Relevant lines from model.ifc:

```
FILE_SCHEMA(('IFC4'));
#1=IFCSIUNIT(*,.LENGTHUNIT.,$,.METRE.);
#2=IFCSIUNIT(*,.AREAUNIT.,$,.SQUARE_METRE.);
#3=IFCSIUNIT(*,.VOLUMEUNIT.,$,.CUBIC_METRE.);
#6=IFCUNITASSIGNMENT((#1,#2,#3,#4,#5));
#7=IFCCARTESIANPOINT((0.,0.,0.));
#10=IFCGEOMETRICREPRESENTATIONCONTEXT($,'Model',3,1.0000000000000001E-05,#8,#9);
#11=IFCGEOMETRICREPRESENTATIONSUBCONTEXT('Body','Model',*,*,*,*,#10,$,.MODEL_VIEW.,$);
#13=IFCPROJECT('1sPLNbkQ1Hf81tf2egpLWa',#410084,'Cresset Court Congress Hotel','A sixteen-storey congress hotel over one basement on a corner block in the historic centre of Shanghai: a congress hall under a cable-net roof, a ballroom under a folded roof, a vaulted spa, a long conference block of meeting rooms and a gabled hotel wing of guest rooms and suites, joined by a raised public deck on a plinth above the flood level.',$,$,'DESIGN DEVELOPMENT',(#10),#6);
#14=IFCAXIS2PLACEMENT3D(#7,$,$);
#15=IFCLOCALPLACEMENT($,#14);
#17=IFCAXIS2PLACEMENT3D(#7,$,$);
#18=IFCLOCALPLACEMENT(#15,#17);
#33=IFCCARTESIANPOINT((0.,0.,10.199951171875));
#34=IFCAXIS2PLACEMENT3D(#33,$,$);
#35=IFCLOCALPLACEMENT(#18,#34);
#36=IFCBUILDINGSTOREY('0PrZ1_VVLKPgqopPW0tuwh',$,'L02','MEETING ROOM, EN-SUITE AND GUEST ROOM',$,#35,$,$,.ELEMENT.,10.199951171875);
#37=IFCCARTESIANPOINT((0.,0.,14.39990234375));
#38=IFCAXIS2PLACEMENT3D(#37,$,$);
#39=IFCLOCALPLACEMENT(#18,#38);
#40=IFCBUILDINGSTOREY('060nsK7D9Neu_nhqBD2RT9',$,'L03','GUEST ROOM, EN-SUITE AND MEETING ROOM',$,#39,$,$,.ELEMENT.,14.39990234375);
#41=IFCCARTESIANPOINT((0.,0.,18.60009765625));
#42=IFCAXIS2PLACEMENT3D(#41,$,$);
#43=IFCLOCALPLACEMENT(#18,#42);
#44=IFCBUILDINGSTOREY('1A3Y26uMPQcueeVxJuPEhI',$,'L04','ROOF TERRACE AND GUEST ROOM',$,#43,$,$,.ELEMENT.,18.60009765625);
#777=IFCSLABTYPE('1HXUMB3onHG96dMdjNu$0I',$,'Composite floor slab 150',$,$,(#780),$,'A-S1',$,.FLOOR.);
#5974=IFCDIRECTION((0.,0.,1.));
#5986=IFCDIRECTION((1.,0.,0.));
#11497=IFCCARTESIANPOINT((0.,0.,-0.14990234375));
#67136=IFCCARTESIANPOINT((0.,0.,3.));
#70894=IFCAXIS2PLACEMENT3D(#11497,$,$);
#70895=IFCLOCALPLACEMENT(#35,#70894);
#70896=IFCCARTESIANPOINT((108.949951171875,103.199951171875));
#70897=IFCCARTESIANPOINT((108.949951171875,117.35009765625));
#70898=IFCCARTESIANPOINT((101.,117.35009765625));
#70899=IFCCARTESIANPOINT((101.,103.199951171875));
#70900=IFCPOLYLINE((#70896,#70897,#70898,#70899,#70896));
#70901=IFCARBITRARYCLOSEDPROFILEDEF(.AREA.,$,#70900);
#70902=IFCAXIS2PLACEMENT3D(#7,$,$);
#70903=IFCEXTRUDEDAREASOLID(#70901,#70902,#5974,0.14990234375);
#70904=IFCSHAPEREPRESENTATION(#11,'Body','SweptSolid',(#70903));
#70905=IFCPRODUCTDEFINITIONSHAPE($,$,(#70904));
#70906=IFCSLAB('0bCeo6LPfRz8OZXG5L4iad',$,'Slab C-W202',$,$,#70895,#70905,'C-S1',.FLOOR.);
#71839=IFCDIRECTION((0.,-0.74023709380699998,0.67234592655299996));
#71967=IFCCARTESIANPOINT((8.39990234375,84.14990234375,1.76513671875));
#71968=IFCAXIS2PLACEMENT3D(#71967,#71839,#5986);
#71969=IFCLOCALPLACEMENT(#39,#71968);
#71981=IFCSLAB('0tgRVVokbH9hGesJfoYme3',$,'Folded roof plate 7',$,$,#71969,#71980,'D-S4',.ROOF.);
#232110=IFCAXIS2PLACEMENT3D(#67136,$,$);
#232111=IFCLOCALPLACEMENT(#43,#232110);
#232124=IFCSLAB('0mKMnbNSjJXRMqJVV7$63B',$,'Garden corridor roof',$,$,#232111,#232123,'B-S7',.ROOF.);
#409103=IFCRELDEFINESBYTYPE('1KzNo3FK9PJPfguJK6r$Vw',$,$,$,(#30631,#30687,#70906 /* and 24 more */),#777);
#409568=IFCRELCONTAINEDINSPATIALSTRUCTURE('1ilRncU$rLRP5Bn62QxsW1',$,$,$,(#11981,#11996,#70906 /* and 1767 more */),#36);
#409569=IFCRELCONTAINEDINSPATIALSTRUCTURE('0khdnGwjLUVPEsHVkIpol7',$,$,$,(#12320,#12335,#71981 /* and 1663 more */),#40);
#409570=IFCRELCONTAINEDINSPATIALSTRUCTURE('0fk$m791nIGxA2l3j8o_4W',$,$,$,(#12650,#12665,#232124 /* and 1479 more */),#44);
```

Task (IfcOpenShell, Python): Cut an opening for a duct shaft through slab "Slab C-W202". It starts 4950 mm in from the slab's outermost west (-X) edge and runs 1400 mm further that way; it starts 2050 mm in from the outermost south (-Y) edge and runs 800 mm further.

```python
import numpy as np
import ifcopenshell
import ifcopenshell.api.feature
import ifcopenshell.api.geometry
import ifcopenshell.api.root
import ifcopenshell.geom
import ifcopenshell.util.placement
import ifcopenshell.util.representation
import ifcopenshell.util.shape
import ifcopenshell.util.unit

model = ifcopenshell.open("model.ifc")
unit_scale = ifcopenshell.util.unit.calculate_unit_scale(model)
settings = ifcopenshell.geom.settings()


def volume(element):
    """Net volume in cubic metres, openings subtracted."""
    shape = ifcopenshell.geom.create_shape(settings, element)
    return ifcopenshell.util.shape.get_volume(shape.geometry)


slab = model.by_id(70906)
before = volume(slab)

# Extent in the slab's own axes, in metres. The edges named are its -X and -Y sides.
slab_shape = ifcopenshell.geom.create_shape(settings, slab)
vertices = ifcopenshell.util.shape.get_vertices(slab_shape.geometry)
x_min, y_min, bottom = vertices.min(axis=0)
top = vertices[:, 2].max()

opening = ifcopenshell.api.root.create_entity(model, ifc_class="IfcOpeningElement", name="Duct shaft opening", predefined_type="OPENING")
context = ifcopenshell.util.representation.get_context(model, "Model", "Body", "MODEL_VIEW")
width, depth = 1.4, 0.8
outline = [(0.0, 0.0), (width, 0.0), (width, depth), (0.0, depth), (0.0, 0.0)]
# Overshoot both faces by 50 mm so the cut is clean.
shape = ifcopenshell.api.geometry.add_slab_representation(
    model, context=context, depth=top - bottom + 0.1, polyline=outline
)
ifcopenshell.api.geometry.assign_representation(model, product=opening, representation=shape)

matrix = ifcopenshell.util.placement.get_local_placement(slab.ObjectPlacement)
matrix[:, 3] = matrix @ np.append(np.array([x_min + 4.95, y_min + 2.05, bottom - 0.05]) / unit_scale, 1.0)
ifcopenshell.api.geometry.edit_object_placement(model, product=opening, matrix=matrix, is_si=False)
ifcopenshell.api.feature.add_feature(model, feature=opening, element=slab)

after = volume(slab)

print(f"slab volume {before:.3f} -> {after:.3f} m3")

model.write("model-out.ifc")
```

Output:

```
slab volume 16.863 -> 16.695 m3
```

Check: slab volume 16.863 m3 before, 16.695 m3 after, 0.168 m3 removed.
